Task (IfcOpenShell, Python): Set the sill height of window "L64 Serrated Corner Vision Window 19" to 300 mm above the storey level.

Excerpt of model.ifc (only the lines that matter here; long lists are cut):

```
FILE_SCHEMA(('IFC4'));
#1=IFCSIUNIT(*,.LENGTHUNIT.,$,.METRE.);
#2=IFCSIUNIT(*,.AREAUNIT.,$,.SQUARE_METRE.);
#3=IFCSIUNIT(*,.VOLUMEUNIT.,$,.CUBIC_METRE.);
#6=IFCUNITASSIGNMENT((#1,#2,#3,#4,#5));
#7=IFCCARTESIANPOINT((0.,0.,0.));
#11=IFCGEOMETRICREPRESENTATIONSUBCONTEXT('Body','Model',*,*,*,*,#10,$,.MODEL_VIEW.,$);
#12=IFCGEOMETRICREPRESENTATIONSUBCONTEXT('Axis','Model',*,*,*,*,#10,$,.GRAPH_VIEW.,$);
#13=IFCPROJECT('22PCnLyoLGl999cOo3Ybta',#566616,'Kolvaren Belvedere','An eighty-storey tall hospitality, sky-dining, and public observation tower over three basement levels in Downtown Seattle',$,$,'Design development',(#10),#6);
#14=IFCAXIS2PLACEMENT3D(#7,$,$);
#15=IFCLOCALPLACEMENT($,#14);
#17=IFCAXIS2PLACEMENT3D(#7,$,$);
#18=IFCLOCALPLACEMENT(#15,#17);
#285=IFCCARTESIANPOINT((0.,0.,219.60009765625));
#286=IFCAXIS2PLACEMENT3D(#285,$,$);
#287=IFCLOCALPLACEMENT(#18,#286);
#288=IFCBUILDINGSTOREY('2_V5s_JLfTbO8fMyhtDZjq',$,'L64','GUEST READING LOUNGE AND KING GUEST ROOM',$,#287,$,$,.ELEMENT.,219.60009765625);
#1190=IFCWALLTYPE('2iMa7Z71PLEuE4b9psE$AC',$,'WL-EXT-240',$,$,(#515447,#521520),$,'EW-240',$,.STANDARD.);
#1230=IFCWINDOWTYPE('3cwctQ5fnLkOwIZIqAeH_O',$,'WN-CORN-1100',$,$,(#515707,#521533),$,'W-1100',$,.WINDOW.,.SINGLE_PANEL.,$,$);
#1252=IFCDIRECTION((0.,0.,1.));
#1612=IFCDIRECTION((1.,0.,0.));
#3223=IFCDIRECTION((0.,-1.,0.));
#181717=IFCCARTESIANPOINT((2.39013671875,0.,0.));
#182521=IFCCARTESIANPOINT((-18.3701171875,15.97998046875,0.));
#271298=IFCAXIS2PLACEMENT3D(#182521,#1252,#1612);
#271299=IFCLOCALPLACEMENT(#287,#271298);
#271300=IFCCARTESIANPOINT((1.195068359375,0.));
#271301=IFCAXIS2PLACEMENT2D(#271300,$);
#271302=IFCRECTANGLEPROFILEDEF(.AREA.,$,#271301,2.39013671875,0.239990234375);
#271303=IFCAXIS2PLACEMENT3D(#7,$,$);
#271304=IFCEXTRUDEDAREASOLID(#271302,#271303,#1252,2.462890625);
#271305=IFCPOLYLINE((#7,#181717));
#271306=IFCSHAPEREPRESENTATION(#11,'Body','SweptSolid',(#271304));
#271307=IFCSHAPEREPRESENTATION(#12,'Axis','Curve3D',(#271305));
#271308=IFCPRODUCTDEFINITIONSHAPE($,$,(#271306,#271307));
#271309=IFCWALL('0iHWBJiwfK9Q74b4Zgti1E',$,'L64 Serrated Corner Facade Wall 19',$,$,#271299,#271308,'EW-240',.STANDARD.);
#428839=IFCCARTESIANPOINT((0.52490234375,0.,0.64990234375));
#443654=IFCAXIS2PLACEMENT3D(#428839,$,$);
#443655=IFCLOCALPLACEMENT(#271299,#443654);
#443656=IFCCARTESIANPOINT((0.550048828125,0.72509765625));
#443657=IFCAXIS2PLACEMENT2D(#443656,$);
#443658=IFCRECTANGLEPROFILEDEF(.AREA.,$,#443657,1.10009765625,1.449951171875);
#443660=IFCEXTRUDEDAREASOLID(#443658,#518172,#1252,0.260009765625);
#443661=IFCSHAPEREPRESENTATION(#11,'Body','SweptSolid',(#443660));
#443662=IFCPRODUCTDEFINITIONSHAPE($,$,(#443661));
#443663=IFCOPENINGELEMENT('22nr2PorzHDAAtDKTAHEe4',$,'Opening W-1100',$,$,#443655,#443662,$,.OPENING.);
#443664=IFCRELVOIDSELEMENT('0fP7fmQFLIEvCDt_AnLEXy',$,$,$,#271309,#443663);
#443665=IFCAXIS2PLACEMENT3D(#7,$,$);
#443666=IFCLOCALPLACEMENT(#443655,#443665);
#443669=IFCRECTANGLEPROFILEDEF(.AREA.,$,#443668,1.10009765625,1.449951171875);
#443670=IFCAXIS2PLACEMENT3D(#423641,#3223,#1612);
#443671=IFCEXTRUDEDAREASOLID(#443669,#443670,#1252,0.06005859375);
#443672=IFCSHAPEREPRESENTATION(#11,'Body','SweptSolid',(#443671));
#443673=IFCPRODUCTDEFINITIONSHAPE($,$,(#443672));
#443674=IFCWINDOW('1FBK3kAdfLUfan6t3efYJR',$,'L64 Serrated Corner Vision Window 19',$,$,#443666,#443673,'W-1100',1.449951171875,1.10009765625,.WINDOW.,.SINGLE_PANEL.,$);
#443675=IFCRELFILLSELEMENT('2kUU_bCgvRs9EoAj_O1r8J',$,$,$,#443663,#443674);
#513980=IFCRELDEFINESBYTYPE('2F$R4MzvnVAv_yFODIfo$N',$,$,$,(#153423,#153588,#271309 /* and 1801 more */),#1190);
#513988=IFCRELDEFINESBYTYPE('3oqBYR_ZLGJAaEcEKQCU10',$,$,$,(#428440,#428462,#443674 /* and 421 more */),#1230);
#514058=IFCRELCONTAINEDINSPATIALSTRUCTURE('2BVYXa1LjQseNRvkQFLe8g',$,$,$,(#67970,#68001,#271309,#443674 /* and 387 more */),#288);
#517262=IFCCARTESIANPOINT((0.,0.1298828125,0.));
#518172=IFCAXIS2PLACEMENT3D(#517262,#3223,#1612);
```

```python
import numpy as np
import ifcopenshell
import ifcopenshell.api.geometry
import ifcopenshell.geom
import ifcopenshell.util.element
import ifcopenshell.util.placement
import ifcopenshell.util.shape
import ifcopenshell.util.unit

model = ifcopenshell.open("model.ifc")
unit_scale = ifcopenshell.util.unit.calculate_unit_scale(model)

window = model.by_guid("1FBK3kAdfLUfan6t3efYJR")
opening = window.FillsVoids[0].RelatingOpeningElement
storey = ifcopenshell.util.element.get_container(window, ifc_class="IfcBuildingStorey")
level = ifcopenshell.util.placement.get_local_placement(storey.ObjectPlacement)[2, 3]

# The opening's origin need not be at the sill, so measure its lowest point.
shape = ifcopenshell.geom.create_shape(ifcopenshell.geom.settings(), opening)
bottom = ifcopenshell.util.shape.get_shape_bottom_elevation(shape, shape.geometry) / unit_scale
dz = level + 0.3 / unit_scale - bottom

shift = np.array([0.0, 0.0, dz])
# The window is placed relative to its opening, so it follows when the opening moves.
matrix = ifcopenshell.util.placement.get_local_placement(opening.ObjectPlacement)
matrix[:3, 3] += shift
ifcopenshell.api.geometry.edit_object_placement(
    model, product=opening, matrix=matrix, is_si=False, should_transform_children=True
)

print(f"moved by {dz * unit_scale:+.3f} m")

model.write("model-out.ifc")
```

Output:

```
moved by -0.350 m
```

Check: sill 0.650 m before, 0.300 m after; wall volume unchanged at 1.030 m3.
